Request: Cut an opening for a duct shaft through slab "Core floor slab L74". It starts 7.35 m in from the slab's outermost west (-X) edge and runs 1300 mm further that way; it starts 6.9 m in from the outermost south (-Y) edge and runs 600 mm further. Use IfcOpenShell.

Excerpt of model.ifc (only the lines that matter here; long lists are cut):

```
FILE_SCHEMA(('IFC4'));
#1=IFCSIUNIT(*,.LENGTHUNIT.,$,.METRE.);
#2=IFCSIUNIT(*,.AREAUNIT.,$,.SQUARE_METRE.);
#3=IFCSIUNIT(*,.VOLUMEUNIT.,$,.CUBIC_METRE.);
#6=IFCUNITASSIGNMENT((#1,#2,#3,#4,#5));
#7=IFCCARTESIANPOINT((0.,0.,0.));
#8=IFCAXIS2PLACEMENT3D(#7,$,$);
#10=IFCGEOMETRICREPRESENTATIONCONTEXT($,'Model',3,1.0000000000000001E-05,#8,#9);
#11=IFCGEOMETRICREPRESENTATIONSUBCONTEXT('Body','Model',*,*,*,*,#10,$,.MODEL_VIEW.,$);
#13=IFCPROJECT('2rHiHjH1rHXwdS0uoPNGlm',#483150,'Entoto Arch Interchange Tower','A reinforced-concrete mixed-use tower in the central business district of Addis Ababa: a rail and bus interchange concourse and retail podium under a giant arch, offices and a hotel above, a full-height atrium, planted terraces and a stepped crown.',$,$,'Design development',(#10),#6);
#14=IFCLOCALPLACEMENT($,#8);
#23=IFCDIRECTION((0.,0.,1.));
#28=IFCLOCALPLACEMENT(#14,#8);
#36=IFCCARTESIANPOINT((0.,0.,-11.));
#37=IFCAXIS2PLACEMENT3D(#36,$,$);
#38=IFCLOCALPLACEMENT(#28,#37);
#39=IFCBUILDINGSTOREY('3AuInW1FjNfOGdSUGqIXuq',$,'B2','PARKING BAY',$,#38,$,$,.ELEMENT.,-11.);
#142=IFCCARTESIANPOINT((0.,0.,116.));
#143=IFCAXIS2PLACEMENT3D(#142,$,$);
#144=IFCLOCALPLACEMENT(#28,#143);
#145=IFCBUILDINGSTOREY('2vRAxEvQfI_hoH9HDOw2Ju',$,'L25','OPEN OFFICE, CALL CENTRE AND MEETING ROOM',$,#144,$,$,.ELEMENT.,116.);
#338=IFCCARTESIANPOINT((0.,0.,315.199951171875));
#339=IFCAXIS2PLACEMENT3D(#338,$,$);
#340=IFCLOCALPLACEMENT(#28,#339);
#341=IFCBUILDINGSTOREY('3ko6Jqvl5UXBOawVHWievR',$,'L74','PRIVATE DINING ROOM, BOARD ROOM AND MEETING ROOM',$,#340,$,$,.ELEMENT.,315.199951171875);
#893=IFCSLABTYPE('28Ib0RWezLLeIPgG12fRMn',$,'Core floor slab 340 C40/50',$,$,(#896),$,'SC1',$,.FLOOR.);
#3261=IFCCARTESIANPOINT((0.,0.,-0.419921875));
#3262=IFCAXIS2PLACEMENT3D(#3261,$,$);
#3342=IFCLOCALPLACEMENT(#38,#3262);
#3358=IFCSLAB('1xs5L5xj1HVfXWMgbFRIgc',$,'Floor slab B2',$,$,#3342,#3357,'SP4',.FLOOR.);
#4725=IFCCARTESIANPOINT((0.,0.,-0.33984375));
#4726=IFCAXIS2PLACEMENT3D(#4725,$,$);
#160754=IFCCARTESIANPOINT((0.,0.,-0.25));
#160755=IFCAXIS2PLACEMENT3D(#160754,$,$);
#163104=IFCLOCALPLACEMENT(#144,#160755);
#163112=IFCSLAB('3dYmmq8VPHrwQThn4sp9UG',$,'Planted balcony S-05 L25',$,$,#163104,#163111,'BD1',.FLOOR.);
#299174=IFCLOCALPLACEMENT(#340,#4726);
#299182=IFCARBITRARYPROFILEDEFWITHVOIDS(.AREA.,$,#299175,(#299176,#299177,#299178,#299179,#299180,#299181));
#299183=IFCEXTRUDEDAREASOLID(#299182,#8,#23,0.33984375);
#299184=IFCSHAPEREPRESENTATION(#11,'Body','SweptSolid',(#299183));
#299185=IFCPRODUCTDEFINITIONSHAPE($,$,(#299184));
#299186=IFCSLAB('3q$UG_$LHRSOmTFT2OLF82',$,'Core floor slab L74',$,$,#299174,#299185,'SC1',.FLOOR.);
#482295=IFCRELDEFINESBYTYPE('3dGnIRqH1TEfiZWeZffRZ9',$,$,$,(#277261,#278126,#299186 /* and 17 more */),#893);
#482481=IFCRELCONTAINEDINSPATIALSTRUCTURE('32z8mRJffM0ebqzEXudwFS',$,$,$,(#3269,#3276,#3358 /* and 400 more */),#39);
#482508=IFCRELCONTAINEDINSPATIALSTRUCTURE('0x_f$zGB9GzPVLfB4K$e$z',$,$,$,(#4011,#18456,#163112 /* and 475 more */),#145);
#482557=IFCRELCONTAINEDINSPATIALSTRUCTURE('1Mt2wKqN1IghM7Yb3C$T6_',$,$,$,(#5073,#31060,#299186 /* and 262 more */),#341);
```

```python
import numpy as np
import ifcopenshell
import ifcopenshell.api.feature
import ifcopenshell.api.geometry
import ifcopenshell.api.root
import ifcopenshell.geom
import ifcopenshell.util.placement
import ifcopenshell.util.representation
import ifcopenshell.util.shape
import ifcopenshell.util.unit

model = ifcopenshell.open("model.ifc")
unit_scale = ifcopenshell.util.unit.calculate_unit_scale(model)
settings = ifcopenshell.geom.settings()


def volume(element):
    """Net volume in cubic metres, openings subtracted."""
    shape = ifcopenshell.geom.create_shape(settings, element)
    return ifcopenshell.util.shape.get_volume(shape.geometry)


slab = model.by_guid("3q$UG_$LHRSOmTFT2OLF82")
before = volume(slab)

# Extent in the slab's own axes, in metres. The edges named are its -X and -Y sides.
slab_shape = ifcopenshell.geom.create_shape(settings, slab)
vertices = ifcopenshell.util.shape.get_vertices(slab_shape.geometry)
x_min, y_min, bottom = vertices.min(axis=0)
top = vertices[:, 2].max()

opening = ifcopenshell.api.root.create_entity(model, ifc_class="IfcOpeningElement", name="Duct shaft opening", predefined_type="OPENING")
context = ifcopenshell.util.representation.get_context(model, "Model", "Body", "MODEL_VIEW")
width, depth = 1.3, 0.6
outline = [(0.0, 0.0), (width, 0.0), (width, depth), (0.0, depth), (0.0, 0.0)]
# Overshoot both faces by 50 mm so the cut is clean.
shape = ifcopenshell.api.geometry.add_slab_representation(
    model, context=context, depth=top - bottom + 0.1, polyline=outline
)
ifcopenshell.api.geometry.assign_representation(model, product=opening, representation=shape)

matrix = ifcopenshell.util.placement.get_local_placement(slab.ObjectPlacement)
matrix[:, 3] = matrix @ np.append(np.array([x_min + 7.35, y_min + 6.9, bottom - 0.05]) / unit_scale, 1.0)
ifcopenshell.api.geometry.edit_object_placement(model, product=opening, matrix=matrix, is_si=False)
ifcopenshell.api.feature.add_feature(model, feature=opening, element=slab)

after = volume(slab)

print(f"slab volume {before:.3f} -> {after:.3f} m3")

model.write("model-out.ifc")
```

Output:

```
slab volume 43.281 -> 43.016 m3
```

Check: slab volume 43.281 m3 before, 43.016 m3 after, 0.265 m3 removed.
